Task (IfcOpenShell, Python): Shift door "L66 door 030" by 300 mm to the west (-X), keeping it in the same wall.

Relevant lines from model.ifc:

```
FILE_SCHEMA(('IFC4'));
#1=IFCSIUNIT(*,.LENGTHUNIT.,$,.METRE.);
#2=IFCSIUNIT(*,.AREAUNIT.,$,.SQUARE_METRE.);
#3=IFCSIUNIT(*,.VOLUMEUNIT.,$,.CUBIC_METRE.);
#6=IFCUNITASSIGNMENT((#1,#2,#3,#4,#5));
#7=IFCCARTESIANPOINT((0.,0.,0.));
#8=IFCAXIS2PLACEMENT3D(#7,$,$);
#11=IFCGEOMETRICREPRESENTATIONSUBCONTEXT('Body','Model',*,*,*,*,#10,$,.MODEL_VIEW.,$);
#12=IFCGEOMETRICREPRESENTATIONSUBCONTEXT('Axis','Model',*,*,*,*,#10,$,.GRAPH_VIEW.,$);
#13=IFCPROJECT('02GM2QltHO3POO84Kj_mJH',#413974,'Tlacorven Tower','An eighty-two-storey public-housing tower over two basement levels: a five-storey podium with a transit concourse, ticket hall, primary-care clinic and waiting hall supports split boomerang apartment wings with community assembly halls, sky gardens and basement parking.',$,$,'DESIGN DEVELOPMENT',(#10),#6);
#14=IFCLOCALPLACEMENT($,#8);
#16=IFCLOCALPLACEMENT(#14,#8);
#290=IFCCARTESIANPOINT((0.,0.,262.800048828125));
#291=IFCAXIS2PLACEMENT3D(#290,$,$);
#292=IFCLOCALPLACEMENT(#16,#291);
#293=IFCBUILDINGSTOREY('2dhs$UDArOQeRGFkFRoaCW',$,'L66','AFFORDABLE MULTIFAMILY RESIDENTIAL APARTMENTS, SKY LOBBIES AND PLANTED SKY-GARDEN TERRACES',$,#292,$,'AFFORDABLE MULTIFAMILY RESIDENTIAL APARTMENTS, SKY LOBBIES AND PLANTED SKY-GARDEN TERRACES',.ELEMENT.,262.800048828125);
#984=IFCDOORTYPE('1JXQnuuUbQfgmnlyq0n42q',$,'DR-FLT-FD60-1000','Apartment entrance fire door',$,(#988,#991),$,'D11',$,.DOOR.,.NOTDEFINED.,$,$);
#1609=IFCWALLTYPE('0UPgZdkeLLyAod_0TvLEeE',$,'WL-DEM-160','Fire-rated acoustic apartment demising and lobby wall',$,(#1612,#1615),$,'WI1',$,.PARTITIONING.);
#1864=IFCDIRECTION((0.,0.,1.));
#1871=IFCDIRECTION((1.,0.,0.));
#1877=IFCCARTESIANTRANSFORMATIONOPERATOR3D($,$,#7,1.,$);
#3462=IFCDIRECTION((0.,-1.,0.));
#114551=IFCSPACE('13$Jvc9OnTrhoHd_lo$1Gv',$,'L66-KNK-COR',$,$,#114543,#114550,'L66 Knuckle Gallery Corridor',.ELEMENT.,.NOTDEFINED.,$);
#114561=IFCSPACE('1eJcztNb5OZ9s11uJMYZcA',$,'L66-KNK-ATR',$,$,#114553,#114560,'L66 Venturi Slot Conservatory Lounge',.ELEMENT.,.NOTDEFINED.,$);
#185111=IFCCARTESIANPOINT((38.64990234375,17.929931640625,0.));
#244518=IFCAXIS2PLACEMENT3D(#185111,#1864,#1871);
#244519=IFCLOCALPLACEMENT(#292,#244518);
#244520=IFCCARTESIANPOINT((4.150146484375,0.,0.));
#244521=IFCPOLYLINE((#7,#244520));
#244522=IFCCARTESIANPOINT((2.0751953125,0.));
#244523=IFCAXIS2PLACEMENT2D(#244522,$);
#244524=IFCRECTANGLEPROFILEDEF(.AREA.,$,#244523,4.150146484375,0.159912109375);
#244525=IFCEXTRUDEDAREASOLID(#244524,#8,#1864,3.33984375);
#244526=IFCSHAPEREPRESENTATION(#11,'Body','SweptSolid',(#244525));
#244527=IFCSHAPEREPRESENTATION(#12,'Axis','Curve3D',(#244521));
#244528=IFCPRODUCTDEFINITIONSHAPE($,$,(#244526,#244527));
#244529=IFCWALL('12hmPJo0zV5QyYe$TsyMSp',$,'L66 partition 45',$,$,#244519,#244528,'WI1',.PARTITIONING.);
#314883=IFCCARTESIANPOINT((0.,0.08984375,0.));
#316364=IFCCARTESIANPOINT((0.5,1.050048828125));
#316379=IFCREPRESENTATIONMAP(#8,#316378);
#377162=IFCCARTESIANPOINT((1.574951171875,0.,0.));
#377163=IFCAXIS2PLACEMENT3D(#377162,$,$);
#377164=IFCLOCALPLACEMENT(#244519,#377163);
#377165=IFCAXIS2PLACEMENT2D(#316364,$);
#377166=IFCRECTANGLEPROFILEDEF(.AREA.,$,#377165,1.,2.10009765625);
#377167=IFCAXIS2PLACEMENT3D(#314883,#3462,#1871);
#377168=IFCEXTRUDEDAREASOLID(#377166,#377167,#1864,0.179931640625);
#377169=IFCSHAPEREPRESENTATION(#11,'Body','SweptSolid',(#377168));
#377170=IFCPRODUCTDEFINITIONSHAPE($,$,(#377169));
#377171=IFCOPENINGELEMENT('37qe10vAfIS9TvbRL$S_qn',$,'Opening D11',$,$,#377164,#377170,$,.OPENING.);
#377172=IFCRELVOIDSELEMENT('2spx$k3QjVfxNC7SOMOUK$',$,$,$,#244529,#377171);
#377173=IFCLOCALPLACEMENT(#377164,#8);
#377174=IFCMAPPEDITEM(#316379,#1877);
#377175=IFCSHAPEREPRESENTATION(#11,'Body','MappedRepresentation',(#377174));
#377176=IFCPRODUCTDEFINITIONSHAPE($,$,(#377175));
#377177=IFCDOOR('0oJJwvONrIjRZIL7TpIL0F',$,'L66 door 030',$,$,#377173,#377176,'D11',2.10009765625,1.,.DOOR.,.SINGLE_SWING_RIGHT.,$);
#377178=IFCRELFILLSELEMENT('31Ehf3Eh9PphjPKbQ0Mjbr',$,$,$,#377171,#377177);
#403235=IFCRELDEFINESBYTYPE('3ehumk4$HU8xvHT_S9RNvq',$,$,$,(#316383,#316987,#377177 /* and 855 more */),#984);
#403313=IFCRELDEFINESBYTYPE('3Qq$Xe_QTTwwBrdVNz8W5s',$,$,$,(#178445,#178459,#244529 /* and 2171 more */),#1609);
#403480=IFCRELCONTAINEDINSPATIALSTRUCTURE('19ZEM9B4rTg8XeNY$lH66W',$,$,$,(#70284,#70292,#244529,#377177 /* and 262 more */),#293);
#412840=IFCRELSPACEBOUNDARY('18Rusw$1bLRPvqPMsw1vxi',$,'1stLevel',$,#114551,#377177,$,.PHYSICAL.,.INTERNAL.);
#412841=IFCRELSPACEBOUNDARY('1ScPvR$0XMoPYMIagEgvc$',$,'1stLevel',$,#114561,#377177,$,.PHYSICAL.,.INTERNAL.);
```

```python
import ifcopenshell
import ifcopenshell.api.geometry
import ifcopenshell.util.placement
import ifcopenshell.util.unit

model = ifcopenshell.open("model.ifc")
unit_scale = ifcopenshell.util.unit.calculate_unit_scale(model)

door = model.by_guid("0oJJwvONrIjRZIL7TpIL0F")
opening = door.FillsVoids[0].RelatingOpeningElement
wall = opening.VoidsElements[0].RelatingBuildingElement

wall_matrix = ifcopenshell.util.placement.get_local_placement(wall.ObjectPlacement)
shift = wall_matrix[:3, 0] * -0.3 / unit_scale
before = ifcopenshell.util.placement.get_local_placement(door.ObjectPlacement)[:3, 3].copy()

# The door is placed relative to its opening, so it follows when the opening moves.
matrix = ifcopenshell.util.placement.get_local_placement(opening.ObjectPlacement)
matrix[:3, 3] += shift
ifcopenshell.api.geometry.edit_object_placement(
    model, product=opening, matrix=matrix, is_si=False, should_transform_children=True
)

after = ifcopenshell.util.placement.get_local_placement(door.ObjectPlacement)[:3, 3]
print("door moved by", (after - before).round(3) + 0.0)

model.write("model_edited.ifc")
```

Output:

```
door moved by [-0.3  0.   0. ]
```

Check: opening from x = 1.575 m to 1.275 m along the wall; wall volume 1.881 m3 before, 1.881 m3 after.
